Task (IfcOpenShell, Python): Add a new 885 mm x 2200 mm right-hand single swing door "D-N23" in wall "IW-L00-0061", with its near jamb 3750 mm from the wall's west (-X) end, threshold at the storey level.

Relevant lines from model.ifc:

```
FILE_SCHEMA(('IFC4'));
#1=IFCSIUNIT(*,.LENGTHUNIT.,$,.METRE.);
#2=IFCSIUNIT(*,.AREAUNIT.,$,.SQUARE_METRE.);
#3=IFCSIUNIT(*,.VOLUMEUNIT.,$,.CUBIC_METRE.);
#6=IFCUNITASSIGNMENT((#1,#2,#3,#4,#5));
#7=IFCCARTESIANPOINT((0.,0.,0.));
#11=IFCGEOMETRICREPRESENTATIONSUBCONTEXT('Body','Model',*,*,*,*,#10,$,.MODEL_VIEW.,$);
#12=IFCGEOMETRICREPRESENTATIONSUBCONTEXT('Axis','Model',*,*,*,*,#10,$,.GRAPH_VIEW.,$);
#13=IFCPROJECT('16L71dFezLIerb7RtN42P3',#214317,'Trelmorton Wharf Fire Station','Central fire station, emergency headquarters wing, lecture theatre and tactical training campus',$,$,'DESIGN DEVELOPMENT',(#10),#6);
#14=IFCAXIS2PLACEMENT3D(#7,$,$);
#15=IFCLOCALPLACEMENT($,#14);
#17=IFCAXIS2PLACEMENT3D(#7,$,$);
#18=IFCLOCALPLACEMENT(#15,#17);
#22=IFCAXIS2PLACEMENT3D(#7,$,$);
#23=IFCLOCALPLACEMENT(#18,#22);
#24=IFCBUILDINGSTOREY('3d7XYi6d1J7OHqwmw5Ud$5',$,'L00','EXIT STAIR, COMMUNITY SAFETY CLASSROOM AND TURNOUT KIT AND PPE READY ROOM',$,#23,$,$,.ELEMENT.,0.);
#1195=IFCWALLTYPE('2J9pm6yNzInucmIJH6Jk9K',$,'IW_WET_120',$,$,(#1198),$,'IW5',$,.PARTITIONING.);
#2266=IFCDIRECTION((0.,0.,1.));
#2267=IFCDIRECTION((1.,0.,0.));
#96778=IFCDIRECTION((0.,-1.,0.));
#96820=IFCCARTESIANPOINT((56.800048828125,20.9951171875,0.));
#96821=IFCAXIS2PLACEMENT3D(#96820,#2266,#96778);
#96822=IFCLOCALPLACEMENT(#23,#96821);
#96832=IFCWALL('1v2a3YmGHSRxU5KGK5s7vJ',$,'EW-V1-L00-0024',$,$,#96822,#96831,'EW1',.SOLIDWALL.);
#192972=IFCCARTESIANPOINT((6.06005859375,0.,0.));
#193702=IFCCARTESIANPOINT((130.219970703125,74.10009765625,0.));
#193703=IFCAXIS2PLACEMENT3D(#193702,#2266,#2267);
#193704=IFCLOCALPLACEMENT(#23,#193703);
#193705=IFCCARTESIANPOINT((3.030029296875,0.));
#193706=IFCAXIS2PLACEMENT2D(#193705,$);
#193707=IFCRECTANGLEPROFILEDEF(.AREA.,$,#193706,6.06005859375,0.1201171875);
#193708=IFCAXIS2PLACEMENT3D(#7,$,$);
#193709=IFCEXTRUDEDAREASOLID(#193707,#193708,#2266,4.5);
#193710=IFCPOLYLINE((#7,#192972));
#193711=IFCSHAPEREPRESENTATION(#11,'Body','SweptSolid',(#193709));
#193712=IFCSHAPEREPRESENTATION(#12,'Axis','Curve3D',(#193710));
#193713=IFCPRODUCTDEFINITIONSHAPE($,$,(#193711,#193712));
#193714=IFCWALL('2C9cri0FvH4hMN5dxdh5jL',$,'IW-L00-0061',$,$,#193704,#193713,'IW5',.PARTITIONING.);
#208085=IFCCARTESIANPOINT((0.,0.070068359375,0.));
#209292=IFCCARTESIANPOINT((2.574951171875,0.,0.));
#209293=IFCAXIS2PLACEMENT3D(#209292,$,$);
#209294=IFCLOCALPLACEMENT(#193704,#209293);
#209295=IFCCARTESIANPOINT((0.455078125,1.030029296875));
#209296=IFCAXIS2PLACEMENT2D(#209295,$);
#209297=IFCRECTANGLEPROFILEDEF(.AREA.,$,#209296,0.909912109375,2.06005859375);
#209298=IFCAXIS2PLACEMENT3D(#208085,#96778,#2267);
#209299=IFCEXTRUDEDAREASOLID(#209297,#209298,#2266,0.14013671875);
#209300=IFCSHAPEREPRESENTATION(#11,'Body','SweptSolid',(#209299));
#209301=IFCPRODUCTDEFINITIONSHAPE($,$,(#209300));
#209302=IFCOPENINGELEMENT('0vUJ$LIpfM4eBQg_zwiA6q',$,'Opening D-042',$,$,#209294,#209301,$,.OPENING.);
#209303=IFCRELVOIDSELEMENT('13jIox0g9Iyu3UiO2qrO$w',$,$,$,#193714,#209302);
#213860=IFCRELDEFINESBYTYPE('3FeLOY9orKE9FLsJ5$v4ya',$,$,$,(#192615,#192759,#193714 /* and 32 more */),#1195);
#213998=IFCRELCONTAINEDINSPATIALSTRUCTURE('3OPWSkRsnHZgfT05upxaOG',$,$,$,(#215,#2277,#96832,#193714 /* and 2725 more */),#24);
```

```python
import numpy as np
import ifcopenshell
import ifcopenshell.api.feature
import ifcopenshell.api.geometry
import ifcopenshell.api.root
import ifcopenshell.api.spatial
import ifcopenshell.geom
import ifcopenshell.util.element
import ifcopenshell.util.placement
import ifcopenshell.util.representation
import ifcopenshell.util.shape
import ifcopenshell.util.unit

model = ifcopenshell.open("model.ifc")
unit_scale = ifcopenshell.util.unit.calculate_unit_scale(model)
settings = ifcopenshell.geom.settings()


def volume(element):
    """Net volume in cubic metres, openings subtracted."""
    shape = ifcopenshell.geom.create_shape(settings, element)
    return ifcopenshell.util.shape.get_volume(shape.geometry)


wall = model.by_guid("2C9cri0FvH4hMN5dxdh5jL")
storey = ifcopenshell.util.element.get_container(wall, ifc_class="IfcBuildingStorey")
context = ifcopenshell.util.representation.get_context(model, "Model", "Body", "MODEL_VIEW")
before = volume(wall)

width, height, from_end, sill = 0.885, 2.2, 3.75, 0.0  # metres

# The wall runs along its own X axis, and the end named is its -X end.
wall_shape = ifcopenshell.geom.create_shape(settings, wall)
x, y, z = ifcopenshell.util.shape.get_vertices(wall_shape.geometry).T
start = x.min() + from_end
face, thickness = float(y.min()), float(y.max() - y.min())
wall_matrix = ifcopenshell.util.placement.get_local_placement(wall.ObjectPlacement)
level = ifcopenshell.util.placement.get_local_placement(storey.ObjectPlacement)[2, 3]


def in_wall(x, y):
    """Placement at x, y metres in the wall's axes, at sill height."""
    matrix = wall_matrix.copy()
    matrix[:, 3] = wall_matrix @ np.array([x / unit_scale, y / unit_scale, 0.0, 1.0])
    matrix[2, 3] = level + sill / unit_scale
    return matrix


# Opening: a box that overshoots both wall faces by 50 mm.
opening = ifcopenshell.api.root.create_entity(model, ifc_class="IfcOpeningElement", predefined_type="OPENING")
box = ifcopenshell.api.geometry.add_wall_representation(
    model, context=context, length=width, height=height, thickness=thickness + 0.1
)
ifcopenshell.api.geometry.assign_representation(model, product=opening, representation=box)
ifcopenshell.api.geometry.edit_object_placement(model, product=opening, matrix=in_wall(start, face - 0.05), is_si=False)
ifcopenshell.api.feature.add_feature(model, feature=opening, element=wall)

door = ifcopenshell.api.root.create_entity(model, ifc_class="IfcDoor", name="D-N23", predefined_type="DOOR")
door.OverallWidth, door.OverallHeight = width / unit_scale, height / unit_scale
door.OperationType = "SINGLE_SWING_RIGHT"
body = ifcopenshell.api.geometry.add_door_representation(
    model,
    context=context,
    overall_width=door.OverallWidth,
    overall_height=door.OverallHeight,
    operation_type="SINGLE_SWING_RIGHT",
    lining_properties={"LiningDepth": thickness / unit_scale, "ThresholdDepth": thickness / unit_scale},
)
ifcopenshell.api.geometry.assign_representation(model, product=door, representation=body)
ifcopenshell.api.spatial.assign_container(model, products=[door], relating_structure=storey)
ifcopenshell.api.feature.add_filling(model, opening=opening, element=door)

# The lining spans the wall, so the door starts at the wall face.
ifcopenshell.api.geometry.edit_object_placement(model, product=door, matrix=in_wall(start, face), is_si=False)

after = volume(wall)

print(f"wall volume {before:.3f} -> {after:.3f} m3")

model.write("model_updated.ifc")
```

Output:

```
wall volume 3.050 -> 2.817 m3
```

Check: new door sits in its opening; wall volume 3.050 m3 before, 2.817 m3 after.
